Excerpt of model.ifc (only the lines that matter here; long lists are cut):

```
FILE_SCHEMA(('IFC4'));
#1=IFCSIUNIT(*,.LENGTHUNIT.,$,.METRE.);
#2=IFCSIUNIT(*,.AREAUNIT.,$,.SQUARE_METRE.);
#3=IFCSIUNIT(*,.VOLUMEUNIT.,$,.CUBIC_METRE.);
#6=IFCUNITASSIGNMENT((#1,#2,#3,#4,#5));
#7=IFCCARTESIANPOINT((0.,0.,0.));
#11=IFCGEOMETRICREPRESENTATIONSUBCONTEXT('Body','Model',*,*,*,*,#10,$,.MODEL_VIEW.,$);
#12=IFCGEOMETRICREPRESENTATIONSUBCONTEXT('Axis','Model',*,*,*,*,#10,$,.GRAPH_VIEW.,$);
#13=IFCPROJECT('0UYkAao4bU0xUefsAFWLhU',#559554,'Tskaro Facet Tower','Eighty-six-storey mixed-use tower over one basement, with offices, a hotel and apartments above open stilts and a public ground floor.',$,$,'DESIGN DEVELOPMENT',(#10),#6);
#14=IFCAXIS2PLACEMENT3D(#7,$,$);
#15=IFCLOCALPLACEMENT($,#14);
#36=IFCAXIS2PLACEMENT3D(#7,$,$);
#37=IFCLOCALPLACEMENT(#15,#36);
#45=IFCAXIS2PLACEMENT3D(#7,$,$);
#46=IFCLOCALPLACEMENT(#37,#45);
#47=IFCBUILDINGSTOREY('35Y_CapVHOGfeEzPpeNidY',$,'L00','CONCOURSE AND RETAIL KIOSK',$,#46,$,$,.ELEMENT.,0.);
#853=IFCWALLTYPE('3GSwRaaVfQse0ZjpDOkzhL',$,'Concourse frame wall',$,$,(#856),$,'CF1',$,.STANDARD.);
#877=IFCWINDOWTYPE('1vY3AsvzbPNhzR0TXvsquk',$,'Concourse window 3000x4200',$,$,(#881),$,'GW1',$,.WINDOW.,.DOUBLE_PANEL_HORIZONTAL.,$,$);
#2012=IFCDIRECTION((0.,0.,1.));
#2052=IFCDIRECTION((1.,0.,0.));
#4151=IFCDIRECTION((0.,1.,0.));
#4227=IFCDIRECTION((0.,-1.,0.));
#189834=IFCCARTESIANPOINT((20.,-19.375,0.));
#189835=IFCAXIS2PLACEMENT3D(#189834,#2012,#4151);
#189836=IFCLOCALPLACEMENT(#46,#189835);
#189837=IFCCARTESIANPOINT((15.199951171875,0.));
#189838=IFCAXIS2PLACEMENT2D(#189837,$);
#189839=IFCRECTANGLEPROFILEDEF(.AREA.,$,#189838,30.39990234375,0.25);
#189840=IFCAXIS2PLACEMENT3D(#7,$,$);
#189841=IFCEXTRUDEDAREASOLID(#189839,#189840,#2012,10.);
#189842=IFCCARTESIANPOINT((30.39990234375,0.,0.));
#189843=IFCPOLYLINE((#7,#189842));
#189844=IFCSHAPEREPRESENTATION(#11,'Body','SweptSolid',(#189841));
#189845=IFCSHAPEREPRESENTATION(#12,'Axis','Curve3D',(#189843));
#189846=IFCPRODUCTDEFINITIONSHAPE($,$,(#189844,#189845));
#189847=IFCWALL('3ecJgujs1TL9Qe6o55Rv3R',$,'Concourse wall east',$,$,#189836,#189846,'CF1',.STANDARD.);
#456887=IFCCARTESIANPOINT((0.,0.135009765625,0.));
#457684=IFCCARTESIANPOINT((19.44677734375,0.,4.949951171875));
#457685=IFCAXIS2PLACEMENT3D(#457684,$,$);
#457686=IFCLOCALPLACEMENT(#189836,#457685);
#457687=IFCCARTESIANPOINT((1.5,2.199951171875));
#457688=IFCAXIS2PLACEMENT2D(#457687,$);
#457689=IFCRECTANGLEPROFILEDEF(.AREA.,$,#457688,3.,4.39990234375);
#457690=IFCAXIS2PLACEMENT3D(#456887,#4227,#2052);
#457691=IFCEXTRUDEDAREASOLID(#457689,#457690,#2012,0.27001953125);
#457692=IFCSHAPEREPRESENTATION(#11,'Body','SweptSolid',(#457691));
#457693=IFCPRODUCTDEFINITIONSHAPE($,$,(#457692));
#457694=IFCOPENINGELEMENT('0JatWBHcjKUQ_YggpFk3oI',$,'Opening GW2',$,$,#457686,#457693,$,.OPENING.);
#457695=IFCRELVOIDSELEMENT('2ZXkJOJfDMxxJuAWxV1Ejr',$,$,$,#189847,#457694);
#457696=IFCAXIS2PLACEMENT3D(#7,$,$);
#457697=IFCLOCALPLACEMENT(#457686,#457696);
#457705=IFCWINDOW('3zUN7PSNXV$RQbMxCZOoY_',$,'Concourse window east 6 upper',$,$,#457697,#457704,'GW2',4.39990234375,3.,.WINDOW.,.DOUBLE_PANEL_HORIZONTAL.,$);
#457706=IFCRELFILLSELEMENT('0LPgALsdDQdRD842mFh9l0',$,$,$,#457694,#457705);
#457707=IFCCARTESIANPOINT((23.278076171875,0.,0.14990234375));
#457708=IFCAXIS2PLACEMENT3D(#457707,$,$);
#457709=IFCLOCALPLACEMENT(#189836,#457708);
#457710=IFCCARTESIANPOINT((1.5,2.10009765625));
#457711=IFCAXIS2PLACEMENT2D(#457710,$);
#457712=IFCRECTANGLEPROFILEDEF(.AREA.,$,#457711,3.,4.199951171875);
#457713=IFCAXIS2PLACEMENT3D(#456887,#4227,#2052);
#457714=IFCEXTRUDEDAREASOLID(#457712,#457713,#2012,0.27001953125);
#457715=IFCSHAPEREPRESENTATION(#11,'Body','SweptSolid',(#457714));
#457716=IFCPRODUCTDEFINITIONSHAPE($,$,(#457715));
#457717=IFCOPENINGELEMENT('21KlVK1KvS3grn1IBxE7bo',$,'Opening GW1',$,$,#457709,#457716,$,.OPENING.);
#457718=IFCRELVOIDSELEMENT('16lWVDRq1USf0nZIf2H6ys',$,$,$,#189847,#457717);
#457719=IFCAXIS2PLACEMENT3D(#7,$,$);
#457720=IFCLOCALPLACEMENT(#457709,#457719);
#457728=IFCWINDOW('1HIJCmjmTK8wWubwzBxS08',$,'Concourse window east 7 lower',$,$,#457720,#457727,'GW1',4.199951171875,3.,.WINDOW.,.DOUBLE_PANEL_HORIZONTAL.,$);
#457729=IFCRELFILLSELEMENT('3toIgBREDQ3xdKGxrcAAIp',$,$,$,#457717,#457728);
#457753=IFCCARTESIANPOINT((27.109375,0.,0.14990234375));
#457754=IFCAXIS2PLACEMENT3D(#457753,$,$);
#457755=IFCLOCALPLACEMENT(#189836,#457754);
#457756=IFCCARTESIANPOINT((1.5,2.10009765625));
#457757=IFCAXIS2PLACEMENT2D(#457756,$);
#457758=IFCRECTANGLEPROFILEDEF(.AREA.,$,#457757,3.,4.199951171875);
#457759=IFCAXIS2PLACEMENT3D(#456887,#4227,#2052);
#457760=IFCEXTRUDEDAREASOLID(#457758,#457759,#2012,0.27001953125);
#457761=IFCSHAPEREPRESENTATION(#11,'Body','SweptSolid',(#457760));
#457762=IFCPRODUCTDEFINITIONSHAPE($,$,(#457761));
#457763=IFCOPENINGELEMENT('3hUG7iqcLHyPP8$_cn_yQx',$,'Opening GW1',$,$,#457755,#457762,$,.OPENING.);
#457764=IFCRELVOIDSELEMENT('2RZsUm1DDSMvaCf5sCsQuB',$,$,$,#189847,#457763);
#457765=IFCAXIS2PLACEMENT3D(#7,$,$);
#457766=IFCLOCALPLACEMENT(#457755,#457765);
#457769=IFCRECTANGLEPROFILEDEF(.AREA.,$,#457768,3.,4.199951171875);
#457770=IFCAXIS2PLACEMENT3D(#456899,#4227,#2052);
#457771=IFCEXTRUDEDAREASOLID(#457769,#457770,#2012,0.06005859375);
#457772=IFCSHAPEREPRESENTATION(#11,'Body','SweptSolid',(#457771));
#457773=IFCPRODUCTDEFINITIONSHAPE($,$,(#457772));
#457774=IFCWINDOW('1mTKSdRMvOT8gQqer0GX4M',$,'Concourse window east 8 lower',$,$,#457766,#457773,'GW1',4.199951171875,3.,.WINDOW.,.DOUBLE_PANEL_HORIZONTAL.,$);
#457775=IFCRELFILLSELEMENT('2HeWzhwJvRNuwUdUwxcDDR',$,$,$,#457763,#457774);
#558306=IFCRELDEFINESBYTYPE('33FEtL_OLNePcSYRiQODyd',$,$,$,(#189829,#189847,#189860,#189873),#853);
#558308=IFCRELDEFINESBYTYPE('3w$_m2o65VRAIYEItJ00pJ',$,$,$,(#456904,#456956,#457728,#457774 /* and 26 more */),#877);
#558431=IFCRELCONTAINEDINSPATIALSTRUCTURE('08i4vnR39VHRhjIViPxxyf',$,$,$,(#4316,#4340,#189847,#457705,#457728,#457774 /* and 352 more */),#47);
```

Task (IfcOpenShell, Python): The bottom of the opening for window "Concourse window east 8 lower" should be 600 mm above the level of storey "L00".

```python
import numpy as np
import ifcopenshell
import ifcopenshell.api.geometry
import ifcopenshell.geom
import ifcopenshell.util.element
import ifcopenshell.util.placement
import ifcopenshell.util.shape
import ifcopenshell.util.unit

model = ifcopenshell.open("model.ifc")
unit_scale = ifcopenshell.util.unit.calculate_unit_scale(model)

window = model.by_id(457774)
opening = window.FillsVoids[0].RelatingOpeningElement
storey = ifcopenshell.util.element.get_container(window, ifc_class="IfcBuildingStorey")
level = ifcopenshell.util.placement.get_local_placement(storey.ObjectPlacement)[2, 3]

# The opening's origin need not be at the sill, so measure its lowest point.
shape = ifcopenshell.geom.create_shape(ifcopenshell.geom.settings(), opening)
bottom = ifcopenshell.util.shape.get_shape_bottom_elevation(shape, shape.geometry) / unit_scale
dz = level + 0.6 / unit_scale - bottom

shift = np.array([0.0, 0.0, dz])
# The window is placed relative to its opening, so it follows when the opening moves.
matrix = ifcopenshell.util.placement.get_local_placement(opening.ObjectPlacement)
matrix[:3, 3] += shift
ifcopenshell.api.geometry.edit_object_placement(
    model, product=opening, matrix=matrix, is_si=False, should_transform_children=True
)

print(f"moved by {dz * unit_scale:+.3f} m")

model.write("model_edited.ifc")
```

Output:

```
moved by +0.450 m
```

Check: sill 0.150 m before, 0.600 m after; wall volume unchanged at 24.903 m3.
